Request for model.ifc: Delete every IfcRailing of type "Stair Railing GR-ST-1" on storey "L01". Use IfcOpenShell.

First a look at what the model holds.

```python
import ifcopenshell
import ifcopenshell.util.element

model = ifcopenshell.open("model.ifc")
print(model.schema)
storey = next(s for s in model.by_type("IfcBuildingStorey") if s.Name == "L01")
railings = [e for e in ifcopenshell.util.element.get_decomposition(storey) if e.is_a("IfcRailing")]
seen = {}
for e in railings:
    element_type = ifcopenshell.util.element.get_type(e)
    name = element_type.Name if element_type not in (None, e) else None
    seen[name] = seen.get(name, 0) + 1
for name, count in sorted(seen.items(), key=str):
    print(count, "x", name)
```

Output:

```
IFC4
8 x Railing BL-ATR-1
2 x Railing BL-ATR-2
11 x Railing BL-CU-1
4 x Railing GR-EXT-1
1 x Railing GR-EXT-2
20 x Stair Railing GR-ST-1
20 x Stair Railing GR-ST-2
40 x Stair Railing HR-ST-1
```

```python
import ifcopenshell
import ifcopenshell.api.root
import ifcopenshell.util.element

model = ifcopenshell.open("model.ifc")

storey = next(s for s in model.by_type("IfcBuildingStorey") if s.Name == "L01")
railings = [e for e in ifcopenshell.util.element.get_decomposition(storey) if e.is_a("IfcRailing")]
targets = [e for e in railings if (t := ifcopenshell.util.element.get_type(e)) not in (None, e) and t.Name == "Stair Railing GR-ST-1"]

for e in targets:
    ifcopenshell.api.root.remove_product(model, product=e)
print(len(targets), "removed")

model.write("model_v2.ifc")
```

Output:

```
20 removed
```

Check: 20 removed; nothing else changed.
